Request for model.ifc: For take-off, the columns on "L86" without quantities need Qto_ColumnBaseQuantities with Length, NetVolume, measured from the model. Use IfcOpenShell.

First a look at what the model holds.

```python
import ifcopenshell
import ifcopenshell.util.element
import ifcopenshell.util.unit

model = ifcopenshell.open("model.ifc")
print(model.schema)
for unit_type in ("LENGTHUNIT", "AREAUNIT", "VOLUMEUNIT"):
    print(unit_type, ifcopenshell.util.unit.calculate_unit_scale(model, unit_type))
storey = next(s for s in model.by_type("IfcBuildingStorey") if s.Name == "L86")
columns = [e for e in ifcopenshell.util.element.get_decomposition(storey) if e.is_a("IfcColumn")]
for e in sorted(columns, key=lambda e: e.id()):
    print(e.id(), e.is_a(), e.Name, list(ifcopenshell.util.element.get_psets(e, qtos_only=True)), sep=" | ")
```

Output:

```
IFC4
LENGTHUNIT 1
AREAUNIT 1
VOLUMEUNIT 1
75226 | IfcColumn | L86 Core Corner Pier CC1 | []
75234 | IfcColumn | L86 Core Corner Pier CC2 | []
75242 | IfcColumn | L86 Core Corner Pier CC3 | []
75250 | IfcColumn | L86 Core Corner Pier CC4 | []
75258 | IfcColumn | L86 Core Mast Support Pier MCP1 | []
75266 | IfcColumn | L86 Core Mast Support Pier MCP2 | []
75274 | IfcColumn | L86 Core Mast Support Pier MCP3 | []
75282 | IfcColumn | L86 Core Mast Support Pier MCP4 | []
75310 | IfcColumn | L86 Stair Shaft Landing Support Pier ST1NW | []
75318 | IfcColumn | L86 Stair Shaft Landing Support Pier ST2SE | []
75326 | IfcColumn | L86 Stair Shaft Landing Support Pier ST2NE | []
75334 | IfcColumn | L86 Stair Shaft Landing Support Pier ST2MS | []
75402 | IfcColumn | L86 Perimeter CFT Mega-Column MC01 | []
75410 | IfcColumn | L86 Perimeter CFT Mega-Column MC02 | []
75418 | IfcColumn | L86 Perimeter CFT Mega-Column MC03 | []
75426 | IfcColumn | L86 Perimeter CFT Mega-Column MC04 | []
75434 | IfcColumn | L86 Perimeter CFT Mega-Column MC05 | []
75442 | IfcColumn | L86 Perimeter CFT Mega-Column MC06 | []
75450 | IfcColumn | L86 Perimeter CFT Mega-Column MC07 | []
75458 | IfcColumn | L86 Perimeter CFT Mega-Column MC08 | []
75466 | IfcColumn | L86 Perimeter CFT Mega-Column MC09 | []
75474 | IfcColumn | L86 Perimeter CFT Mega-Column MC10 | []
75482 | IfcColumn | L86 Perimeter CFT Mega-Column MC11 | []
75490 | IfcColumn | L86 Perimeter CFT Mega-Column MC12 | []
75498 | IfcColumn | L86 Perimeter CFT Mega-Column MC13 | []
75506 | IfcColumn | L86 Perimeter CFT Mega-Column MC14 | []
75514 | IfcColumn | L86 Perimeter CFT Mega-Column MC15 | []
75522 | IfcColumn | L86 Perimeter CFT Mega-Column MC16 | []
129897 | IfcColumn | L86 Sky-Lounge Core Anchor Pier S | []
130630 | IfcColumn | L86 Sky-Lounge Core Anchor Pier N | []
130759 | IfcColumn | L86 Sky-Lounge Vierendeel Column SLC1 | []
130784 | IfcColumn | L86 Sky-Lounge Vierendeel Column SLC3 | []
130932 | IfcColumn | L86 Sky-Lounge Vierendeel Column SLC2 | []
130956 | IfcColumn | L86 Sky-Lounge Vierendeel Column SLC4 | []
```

```python
import ifcopenshell
import ifcopenshell.api.pset
import ifcopenshell.geom
import ifcopenshell.util.element
import ifcopenshell.util.shape
import ifcopenshell.util.unit

model = ifcopenshell.open("model.ifc")
unit_scale = ifcopenshell.util.unit.calculate_unit_scale(model)
volume_scale = ifcopenshell.util.unit.calculate_unit_scale(model, "VOLUMEUNIT")
settings = ifcopenshell.geom.settings()

storey = next(s for s in model.by_type("IfcBuildingStorey") if s.Name == "L86")
columns = [e for e in ifcopenshell.util.element.get_decomposition(storey) if e.is_a("IfcColumn")]

for e in sorted(columns, key=lambda e: e.id()):
    if ifcopenshell.util.element.get_psets(e, qtos_only=True, should_inherit=False):
        continue
    # Geometry comes back in metres, in the element's own axes.
    shape = ifcopenshell.geom.create_shape(settings, e)
    values = {
        "Length": ifcopenshell.util.shape.get_z(shape.geometry) / unit_scale,
        "NetVolume": ifcopenshell.util.shape.get_volume(shape.geometry) / volume_scale,
    }
    qto = ifcopenshell.api.pset.add_qto(model, product=e, name="Qto_ColumnBaseQuantities")
    ifcopenshell.api.pset.edit_qto(model, qto=qto, properties=values)
    print(e.id(), {k: round(v, 3) for k, v in values.items()})

model.write("model_edited.ifc")
```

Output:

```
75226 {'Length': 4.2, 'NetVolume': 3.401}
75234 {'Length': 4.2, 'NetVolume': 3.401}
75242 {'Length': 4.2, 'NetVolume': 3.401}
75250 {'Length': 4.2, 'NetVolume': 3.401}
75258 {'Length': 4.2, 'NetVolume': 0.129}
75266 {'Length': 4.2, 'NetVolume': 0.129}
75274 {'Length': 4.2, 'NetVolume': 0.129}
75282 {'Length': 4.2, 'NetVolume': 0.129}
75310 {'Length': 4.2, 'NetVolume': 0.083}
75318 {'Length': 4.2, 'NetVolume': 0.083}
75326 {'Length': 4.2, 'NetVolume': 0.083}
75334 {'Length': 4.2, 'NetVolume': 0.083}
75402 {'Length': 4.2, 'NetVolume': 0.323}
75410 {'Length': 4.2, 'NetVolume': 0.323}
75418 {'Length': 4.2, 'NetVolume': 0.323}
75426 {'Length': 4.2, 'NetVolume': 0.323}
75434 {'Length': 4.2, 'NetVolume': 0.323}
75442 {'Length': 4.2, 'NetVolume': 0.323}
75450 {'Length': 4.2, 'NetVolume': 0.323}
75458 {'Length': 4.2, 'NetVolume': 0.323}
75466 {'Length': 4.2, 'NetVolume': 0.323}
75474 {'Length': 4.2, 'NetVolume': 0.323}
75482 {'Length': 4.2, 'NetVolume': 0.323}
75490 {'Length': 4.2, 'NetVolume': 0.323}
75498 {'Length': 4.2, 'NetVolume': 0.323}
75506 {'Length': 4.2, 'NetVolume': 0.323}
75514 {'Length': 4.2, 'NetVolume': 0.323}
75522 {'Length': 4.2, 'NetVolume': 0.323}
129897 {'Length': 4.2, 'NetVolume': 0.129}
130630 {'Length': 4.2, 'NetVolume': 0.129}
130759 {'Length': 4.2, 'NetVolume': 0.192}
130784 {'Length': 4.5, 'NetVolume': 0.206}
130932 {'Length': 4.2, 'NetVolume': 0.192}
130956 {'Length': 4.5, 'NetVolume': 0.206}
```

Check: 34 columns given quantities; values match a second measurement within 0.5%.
